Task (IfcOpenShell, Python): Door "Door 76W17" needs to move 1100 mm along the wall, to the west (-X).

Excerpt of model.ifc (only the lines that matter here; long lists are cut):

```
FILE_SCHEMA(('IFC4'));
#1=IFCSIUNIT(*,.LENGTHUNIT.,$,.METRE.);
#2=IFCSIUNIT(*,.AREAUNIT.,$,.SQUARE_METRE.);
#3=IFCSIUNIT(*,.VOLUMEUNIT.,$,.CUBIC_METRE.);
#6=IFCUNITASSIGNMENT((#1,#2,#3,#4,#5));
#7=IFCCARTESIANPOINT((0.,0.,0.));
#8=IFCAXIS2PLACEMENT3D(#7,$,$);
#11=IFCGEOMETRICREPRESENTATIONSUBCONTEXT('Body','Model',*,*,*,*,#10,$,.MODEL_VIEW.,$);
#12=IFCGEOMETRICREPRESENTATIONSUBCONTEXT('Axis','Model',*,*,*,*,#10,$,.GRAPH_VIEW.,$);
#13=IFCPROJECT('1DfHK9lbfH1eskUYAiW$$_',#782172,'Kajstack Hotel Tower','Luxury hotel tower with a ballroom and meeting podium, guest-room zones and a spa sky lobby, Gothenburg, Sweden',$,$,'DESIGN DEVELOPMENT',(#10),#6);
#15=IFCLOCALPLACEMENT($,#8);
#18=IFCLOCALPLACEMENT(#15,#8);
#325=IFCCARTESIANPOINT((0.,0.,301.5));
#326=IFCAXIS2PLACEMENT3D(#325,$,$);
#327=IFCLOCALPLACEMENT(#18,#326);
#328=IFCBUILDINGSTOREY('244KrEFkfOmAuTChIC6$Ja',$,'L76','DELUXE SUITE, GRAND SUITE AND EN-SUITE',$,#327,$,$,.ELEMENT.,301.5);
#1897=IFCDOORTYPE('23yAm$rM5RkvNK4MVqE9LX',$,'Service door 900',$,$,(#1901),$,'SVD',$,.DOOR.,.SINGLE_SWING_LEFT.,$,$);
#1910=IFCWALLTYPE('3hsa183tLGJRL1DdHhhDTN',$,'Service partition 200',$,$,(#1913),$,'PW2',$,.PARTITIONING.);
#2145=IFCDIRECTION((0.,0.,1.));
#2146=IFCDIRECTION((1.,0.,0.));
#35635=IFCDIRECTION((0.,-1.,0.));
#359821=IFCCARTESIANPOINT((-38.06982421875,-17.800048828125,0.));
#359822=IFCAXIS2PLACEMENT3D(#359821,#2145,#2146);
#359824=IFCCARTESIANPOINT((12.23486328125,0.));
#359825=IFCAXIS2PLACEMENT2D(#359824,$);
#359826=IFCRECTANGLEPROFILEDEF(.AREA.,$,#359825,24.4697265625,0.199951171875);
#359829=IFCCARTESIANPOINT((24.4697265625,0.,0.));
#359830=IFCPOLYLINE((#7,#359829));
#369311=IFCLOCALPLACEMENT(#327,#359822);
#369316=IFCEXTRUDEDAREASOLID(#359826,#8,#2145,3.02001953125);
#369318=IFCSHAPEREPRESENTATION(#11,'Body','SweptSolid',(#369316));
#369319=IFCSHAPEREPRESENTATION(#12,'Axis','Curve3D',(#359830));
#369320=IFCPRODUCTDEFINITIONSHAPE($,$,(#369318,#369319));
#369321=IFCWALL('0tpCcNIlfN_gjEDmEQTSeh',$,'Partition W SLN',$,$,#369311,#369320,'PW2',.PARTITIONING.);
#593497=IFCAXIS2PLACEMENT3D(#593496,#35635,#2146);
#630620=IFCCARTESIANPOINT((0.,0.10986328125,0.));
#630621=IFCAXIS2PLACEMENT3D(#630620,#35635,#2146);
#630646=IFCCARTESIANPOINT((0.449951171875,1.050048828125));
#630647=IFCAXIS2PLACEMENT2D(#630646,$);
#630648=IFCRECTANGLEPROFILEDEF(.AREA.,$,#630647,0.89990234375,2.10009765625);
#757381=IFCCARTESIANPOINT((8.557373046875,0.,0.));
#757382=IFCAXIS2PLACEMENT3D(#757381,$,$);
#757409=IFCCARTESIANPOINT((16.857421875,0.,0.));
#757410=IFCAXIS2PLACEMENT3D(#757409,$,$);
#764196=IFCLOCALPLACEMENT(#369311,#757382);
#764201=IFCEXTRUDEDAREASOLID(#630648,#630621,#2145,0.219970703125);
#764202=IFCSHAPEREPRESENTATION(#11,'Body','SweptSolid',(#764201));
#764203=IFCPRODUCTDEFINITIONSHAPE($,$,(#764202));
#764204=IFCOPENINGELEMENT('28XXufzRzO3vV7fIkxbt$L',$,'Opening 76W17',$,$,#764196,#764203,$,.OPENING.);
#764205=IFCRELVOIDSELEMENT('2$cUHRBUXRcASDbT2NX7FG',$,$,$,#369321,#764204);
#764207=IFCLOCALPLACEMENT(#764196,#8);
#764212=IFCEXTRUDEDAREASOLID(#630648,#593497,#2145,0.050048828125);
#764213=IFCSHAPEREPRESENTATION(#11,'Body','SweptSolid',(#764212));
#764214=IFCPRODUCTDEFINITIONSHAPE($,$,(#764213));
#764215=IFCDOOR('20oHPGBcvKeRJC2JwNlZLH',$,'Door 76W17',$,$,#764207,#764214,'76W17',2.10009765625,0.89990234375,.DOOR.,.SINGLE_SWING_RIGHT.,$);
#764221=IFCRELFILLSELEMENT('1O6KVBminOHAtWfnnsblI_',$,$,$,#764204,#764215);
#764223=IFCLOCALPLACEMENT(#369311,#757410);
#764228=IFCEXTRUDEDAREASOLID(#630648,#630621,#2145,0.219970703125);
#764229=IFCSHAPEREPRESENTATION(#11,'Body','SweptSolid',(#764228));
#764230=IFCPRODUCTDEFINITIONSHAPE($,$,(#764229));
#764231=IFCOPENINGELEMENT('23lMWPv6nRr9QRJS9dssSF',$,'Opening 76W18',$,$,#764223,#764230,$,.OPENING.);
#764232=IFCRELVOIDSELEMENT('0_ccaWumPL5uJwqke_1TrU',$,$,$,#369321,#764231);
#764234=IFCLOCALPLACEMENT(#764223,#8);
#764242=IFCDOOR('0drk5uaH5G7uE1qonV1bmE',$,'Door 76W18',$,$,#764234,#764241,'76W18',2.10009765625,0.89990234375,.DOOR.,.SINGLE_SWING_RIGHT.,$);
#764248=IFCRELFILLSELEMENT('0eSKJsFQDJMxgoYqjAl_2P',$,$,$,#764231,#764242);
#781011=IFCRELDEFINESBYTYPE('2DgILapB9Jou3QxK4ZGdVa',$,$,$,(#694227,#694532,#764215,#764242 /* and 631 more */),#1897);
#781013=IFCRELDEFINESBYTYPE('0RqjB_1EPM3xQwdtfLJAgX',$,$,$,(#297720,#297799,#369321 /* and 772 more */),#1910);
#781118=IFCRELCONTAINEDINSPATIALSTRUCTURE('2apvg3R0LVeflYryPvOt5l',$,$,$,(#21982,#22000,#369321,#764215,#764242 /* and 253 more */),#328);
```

```python
import ifcopenshell
import ifcopenshell.api.geometry
import ifcopenshell.util.placement
import ifcopenshell.util.unit

model = ifcopenshell.open("model.ifc")
unit_scale = ifcopenshell.util.unit.calculate_unit_scale(model)

door = model.by_guid("20oHPGBcvKeRJC2JwNlZLH")
opening = door.FillsVoids[0].RelatingOpeningElement
wall = opening.VoidsElements[0].RelatingBuildingElement

wall_matrix = ifcopenshell.util.placement.get_local_placement(wall.ObjectPlacement)
shift = wall_matrix[:3, 0] * -1.1 / unit_scale
before = ifcopenshell.util.placement.get_local_placement(door.ObjectPlacement)[:3, 3].copy()

# The door is placed relative to its opening, so it follows when the opening moves.
matrix = ifcopenshell.util.placement.get_local_placement(opening.ObjectPlacement)
matrix[:3, 3] += shift
ifcopenshell.api.geometry.edit_object_placement(
    model, product=opening, matrix=matrix, is_si=False, should_transform_children=True
)

after = ifcopenshell.util.placement.get_local_placement(door.ObjectPlacement)[:3, 3]
print("door moved by", (after - before).round(3) + 0.0)

model.write("model_v2.ifc")
```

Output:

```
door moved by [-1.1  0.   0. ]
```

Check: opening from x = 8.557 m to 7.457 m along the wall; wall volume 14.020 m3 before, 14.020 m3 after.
